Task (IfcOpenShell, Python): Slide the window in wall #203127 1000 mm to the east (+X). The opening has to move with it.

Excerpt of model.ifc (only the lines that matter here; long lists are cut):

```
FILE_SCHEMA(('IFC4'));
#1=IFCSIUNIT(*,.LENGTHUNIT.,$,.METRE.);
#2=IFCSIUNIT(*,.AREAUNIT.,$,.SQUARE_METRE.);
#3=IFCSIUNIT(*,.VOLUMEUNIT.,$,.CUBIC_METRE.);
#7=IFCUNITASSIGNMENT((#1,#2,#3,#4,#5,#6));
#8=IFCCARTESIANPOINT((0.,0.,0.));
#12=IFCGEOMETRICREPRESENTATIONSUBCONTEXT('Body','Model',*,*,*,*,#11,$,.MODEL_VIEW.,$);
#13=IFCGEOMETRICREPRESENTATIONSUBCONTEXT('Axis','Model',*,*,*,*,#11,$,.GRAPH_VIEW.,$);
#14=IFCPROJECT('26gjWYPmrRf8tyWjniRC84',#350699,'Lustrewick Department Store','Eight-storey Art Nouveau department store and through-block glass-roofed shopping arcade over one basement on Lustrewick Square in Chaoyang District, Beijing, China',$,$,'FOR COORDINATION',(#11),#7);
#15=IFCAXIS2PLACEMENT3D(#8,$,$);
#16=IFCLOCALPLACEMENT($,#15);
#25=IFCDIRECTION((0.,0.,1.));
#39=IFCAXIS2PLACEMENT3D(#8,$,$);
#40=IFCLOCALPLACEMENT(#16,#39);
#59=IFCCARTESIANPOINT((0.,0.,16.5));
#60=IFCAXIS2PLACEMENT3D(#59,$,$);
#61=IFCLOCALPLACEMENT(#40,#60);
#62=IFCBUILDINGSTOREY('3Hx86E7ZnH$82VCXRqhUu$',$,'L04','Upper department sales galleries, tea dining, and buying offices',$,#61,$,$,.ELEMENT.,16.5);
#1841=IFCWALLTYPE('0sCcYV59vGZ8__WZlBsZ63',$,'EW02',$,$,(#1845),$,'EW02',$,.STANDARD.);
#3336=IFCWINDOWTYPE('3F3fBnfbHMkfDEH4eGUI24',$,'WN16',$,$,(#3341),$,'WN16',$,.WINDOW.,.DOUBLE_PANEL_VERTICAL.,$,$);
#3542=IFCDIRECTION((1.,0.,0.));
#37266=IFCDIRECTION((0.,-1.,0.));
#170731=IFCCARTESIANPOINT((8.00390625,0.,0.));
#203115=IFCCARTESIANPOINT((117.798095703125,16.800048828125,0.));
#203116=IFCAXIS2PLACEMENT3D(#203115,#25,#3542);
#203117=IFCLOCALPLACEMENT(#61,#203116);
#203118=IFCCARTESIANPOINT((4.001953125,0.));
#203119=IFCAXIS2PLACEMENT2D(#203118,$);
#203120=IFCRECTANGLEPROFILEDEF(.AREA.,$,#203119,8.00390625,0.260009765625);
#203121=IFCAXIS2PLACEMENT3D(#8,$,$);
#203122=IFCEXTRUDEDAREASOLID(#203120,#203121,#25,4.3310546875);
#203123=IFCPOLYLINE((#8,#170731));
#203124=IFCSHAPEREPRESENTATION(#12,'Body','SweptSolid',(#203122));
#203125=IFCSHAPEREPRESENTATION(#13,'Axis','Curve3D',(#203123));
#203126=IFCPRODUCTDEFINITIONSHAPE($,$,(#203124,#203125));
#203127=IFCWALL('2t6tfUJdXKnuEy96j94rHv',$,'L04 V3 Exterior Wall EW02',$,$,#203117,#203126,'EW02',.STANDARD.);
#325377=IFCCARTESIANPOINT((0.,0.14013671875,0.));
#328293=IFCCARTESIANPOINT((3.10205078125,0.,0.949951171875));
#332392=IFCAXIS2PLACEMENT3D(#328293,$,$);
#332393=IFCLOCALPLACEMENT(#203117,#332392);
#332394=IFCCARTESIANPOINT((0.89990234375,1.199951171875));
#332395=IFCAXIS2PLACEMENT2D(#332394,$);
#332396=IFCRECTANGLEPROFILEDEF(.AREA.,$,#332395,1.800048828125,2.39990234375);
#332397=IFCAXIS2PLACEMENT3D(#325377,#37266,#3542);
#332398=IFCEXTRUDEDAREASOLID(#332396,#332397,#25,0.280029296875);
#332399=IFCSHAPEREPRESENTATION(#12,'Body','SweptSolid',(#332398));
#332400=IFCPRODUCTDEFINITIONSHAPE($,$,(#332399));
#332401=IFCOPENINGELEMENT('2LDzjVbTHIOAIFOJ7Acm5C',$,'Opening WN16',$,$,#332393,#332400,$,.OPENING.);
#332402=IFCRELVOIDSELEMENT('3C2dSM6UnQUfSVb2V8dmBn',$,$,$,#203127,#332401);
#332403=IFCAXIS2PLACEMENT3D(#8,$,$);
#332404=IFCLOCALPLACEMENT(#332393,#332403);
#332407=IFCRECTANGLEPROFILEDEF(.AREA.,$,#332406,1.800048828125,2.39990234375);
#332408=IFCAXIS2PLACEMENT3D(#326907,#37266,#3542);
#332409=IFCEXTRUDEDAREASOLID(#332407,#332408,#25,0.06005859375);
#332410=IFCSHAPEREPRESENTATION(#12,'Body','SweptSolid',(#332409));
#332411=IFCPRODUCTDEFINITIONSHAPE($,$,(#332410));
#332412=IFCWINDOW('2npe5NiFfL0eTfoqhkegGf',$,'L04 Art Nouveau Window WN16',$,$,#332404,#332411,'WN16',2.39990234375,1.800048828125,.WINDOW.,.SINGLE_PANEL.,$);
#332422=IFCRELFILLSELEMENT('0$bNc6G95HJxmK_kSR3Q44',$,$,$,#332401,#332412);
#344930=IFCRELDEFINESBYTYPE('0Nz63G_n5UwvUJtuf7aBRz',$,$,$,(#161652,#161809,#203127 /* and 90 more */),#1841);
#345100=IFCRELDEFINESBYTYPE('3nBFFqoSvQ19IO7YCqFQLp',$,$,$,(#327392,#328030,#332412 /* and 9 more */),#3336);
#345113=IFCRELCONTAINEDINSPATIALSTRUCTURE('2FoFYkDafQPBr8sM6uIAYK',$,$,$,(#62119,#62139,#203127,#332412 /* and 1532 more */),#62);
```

```python
import ifcopenshell
import ifcopenshell.api.geometry
import ifcopenshell.util.placement
import ifcopenshell.util.unit

model = ifcopenshell.open("model.ifc")
unit_scale = ifcopenshell.util.unit.calculate_unit_scale(model)

window = model.by_id(332412)
opening = window.FillsVoids[0].RelatingOpeningElement
wall = opening.VoidsElements[0].RelatingBuildingElement

wall_matrix = ifcopenshell.util.placement.get_local_placement(wall.ObjectPlacement)
shift = wall_matrix[:3, 0] * 1 / unit_scale
before = ifcopenshell.util.placement.get_local_placement(window.ObjectPlacement)[:3, 3].copy()

# The window is placed relative to its opening, so it follows when the opening moves.
matrix = ifcopenshell.util.placement.get_local_placement(opening.ObjectPlacement)
matrix[:3, 3] += shift
ifcopenshell.api.geometry.edit_object_placement(
    model, product=opening, matrix=matrix, is_si=False, should_transform_children=True
)

after = ifcopenshell.util.placement.get_local_placement(window.ObjectPlacement)[:3, 3]
print("window moved by", (after - before).round(3) + 0.0)

model.write("model_edited.ifc")
```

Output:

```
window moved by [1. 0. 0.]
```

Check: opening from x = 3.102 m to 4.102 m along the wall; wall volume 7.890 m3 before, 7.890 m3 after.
